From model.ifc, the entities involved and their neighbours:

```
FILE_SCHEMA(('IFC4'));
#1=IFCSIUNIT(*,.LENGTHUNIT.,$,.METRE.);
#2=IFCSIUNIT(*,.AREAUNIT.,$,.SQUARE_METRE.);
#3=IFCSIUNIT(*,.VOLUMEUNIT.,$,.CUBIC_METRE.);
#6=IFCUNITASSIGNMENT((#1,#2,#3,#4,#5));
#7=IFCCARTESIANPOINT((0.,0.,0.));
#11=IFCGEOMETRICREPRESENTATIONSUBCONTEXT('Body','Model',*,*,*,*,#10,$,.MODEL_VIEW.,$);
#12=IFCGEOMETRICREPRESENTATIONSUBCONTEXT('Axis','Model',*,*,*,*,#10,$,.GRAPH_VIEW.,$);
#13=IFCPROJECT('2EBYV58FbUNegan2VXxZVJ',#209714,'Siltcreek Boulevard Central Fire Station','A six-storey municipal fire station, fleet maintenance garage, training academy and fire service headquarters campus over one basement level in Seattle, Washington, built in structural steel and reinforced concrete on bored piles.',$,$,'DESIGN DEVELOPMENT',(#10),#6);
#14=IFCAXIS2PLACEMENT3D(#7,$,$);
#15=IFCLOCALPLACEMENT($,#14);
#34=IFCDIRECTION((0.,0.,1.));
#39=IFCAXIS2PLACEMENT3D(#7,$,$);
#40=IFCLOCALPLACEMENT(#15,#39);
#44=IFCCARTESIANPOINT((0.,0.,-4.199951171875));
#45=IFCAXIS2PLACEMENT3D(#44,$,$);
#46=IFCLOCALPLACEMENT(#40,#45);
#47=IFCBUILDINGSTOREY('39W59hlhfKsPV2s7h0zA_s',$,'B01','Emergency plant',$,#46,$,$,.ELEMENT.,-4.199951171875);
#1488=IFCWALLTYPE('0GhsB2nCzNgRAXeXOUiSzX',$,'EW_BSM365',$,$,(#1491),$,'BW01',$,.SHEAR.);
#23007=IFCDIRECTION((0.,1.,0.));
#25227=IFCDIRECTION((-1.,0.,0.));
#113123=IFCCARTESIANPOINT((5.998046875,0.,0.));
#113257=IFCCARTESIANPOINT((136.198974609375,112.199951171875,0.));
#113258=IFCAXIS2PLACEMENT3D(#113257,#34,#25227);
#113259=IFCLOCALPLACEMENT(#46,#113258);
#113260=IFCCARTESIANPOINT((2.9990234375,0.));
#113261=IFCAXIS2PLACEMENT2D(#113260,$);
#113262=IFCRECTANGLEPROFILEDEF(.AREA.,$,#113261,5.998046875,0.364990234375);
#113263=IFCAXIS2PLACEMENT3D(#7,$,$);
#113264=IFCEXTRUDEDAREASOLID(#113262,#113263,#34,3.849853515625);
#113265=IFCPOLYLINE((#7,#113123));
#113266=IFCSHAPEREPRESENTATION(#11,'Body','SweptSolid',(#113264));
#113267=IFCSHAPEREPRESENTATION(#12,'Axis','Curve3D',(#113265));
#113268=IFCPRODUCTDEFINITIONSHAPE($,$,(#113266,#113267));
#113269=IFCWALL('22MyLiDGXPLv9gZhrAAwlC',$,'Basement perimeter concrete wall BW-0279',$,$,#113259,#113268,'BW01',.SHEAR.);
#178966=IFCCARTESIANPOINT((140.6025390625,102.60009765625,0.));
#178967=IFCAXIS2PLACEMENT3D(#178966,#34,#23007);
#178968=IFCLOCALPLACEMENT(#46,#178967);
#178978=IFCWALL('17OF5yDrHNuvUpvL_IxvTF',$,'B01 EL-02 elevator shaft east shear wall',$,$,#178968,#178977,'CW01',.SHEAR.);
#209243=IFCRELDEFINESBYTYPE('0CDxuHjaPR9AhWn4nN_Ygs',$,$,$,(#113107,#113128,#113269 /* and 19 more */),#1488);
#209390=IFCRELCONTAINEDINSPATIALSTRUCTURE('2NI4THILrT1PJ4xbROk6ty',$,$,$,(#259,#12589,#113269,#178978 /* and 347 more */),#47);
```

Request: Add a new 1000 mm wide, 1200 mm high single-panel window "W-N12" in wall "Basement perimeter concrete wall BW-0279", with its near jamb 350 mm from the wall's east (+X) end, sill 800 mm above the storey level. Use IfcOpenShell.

```python
import numpy as np
import ifcopenshell
import ifcopenshell.api.feature
import ifcopenshell.api.geometry
import ifcopenshell.api.root
import ifcopenshell.api.spatial
import ifcopenshell.geom
import ifcopenshell.util.element
import ifcopenshell.util.placement
import ifcopenshell.util.representation
import ifcopenshell.util.shape
import ifcopenshell.util.unit

model = ifcopenshell.open("model.ifc")
unit_scale = ifcopenshell.util.unit.calculate_unit_scale(model)
settings = ifcopenshell.geom.settings()


def volume(element):
    """Net volume in cubic metres, openings subtracted."""
    shape = ifcopenshell.geom.create_shape(settings, element)
    return ifcopenshell.util.shape.get_volume(shape.geometry)


wall = model.by_guid("22MyLiDGXPLv9gZhrAAwlC")
storey = ifcopenshell.util.element.get_container(wall, ifc_class="IfcBuildingStorey")
context = ifcopenshell.util.representation.get_context(model, "Model", "Body", "MODEL_VIEW")
before = volume(wall)

width, height, from_end, sill = 1, 1.2, 0.35, 0.8  # metres

# The wall runs along its own X axis, and the end named is its -X end.
wall_shape = ifcopenshell.geom.create_shape(settings, wall)
x, y, z = ifcopenshell.util.shape.get_vertices(wall_shape.geometry).T
start = x.min() + from_end
face, thickness = float(y.min()), float(y.max() - y.min())
wall_matrix = ifcopenshell.util.placement.get_local_placement(wall.ObjectPlacement)
level = ifcopenshell.util.placement.get_local_placement(storey.ObjectPlacement)[2, 3]


def in_wall(x, y):
    """Placement at x, y metres in the wall's axes, at sill height."""
    matrix = wall_matrix.copy()
    matrix[:, 3] = wall_matrix @ np.array([x / unit_scale, y / unit_scale, 0.0, 1.0])
    matrix[2, 3] = level + sill / unit_scale
    return matrix


# Opening: a box that overshoots both wall faces by 50 mm.
opening = ifcopenshell.api.root.create_entity(model, ifc_class="IfcOpeningElement", predefined_type="OPENING")
box = ifcopenshell.api.geometry.add_wall_representation(
    model, context=context, length=width, height=height, thickness=thickness + 0.1
)
ifcopenshell.api.geometry.assign_representation(model, product=opening, representation=box)
ifcopenshell.api.geometry.edit_object_placement(model, product=opening, matrix=in_wall(start, face - 0.05), is_si=False)
ifcopenshell.api.feature.add_feature(model, feature=opening, element=wall)

window = ifcopenshell.api.root.create_entity(model, ifc_class="IfcWindow", name="W-N12", predefined_type="WINDOW")
window.OverallWidth, window.OverallHeight = width / unit_scale, height / unit_scale
window.PartitioningType = "SINGLE_PANEL"
body = ifcopenshell.api.geometry.add_window_representation(
    model,
    context=context,
    overall_width=window.OverallWidth,
    overall_height=window.OverallHeight,
    partition_type="SINGLE_PANEL",
)
ifcopenshell.api.geometry.assign_representation(model, product=window, representation=body)
ifcopenshell.api.spatial.assign_container(model, products=[window], relating_structure=storey)
ifcopenshell.api.feature.add_filling(model, opening=opening, element=window)

# Centre the window in the wall's thickness.
ifcopenshell.api.geometry.edit_object_placement(model, product=window, matrix=in_wall(start, face), is_si=False)
window_shape = ifcopenshell.geom.create_shape(settings, window)
depth = ifcopenshell.util.shape.get_vertices(window_shape.geometry)[:, 1]
offset = face + thickness / 2 - (depth.min() + depth.max()) / 2
ifcopenshell.api.geometry.edit_object_placement(model, product=window, matrix=in_wall(start, offset), is_si=False)

after = volume(wall)

print(f"wall volume {before:.3f} -> {after:.3f} m3")

model.write("model_updated.ifc")
```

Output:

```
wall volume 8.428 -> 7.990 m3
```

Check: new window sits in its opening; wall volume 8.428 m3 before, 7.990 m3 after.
